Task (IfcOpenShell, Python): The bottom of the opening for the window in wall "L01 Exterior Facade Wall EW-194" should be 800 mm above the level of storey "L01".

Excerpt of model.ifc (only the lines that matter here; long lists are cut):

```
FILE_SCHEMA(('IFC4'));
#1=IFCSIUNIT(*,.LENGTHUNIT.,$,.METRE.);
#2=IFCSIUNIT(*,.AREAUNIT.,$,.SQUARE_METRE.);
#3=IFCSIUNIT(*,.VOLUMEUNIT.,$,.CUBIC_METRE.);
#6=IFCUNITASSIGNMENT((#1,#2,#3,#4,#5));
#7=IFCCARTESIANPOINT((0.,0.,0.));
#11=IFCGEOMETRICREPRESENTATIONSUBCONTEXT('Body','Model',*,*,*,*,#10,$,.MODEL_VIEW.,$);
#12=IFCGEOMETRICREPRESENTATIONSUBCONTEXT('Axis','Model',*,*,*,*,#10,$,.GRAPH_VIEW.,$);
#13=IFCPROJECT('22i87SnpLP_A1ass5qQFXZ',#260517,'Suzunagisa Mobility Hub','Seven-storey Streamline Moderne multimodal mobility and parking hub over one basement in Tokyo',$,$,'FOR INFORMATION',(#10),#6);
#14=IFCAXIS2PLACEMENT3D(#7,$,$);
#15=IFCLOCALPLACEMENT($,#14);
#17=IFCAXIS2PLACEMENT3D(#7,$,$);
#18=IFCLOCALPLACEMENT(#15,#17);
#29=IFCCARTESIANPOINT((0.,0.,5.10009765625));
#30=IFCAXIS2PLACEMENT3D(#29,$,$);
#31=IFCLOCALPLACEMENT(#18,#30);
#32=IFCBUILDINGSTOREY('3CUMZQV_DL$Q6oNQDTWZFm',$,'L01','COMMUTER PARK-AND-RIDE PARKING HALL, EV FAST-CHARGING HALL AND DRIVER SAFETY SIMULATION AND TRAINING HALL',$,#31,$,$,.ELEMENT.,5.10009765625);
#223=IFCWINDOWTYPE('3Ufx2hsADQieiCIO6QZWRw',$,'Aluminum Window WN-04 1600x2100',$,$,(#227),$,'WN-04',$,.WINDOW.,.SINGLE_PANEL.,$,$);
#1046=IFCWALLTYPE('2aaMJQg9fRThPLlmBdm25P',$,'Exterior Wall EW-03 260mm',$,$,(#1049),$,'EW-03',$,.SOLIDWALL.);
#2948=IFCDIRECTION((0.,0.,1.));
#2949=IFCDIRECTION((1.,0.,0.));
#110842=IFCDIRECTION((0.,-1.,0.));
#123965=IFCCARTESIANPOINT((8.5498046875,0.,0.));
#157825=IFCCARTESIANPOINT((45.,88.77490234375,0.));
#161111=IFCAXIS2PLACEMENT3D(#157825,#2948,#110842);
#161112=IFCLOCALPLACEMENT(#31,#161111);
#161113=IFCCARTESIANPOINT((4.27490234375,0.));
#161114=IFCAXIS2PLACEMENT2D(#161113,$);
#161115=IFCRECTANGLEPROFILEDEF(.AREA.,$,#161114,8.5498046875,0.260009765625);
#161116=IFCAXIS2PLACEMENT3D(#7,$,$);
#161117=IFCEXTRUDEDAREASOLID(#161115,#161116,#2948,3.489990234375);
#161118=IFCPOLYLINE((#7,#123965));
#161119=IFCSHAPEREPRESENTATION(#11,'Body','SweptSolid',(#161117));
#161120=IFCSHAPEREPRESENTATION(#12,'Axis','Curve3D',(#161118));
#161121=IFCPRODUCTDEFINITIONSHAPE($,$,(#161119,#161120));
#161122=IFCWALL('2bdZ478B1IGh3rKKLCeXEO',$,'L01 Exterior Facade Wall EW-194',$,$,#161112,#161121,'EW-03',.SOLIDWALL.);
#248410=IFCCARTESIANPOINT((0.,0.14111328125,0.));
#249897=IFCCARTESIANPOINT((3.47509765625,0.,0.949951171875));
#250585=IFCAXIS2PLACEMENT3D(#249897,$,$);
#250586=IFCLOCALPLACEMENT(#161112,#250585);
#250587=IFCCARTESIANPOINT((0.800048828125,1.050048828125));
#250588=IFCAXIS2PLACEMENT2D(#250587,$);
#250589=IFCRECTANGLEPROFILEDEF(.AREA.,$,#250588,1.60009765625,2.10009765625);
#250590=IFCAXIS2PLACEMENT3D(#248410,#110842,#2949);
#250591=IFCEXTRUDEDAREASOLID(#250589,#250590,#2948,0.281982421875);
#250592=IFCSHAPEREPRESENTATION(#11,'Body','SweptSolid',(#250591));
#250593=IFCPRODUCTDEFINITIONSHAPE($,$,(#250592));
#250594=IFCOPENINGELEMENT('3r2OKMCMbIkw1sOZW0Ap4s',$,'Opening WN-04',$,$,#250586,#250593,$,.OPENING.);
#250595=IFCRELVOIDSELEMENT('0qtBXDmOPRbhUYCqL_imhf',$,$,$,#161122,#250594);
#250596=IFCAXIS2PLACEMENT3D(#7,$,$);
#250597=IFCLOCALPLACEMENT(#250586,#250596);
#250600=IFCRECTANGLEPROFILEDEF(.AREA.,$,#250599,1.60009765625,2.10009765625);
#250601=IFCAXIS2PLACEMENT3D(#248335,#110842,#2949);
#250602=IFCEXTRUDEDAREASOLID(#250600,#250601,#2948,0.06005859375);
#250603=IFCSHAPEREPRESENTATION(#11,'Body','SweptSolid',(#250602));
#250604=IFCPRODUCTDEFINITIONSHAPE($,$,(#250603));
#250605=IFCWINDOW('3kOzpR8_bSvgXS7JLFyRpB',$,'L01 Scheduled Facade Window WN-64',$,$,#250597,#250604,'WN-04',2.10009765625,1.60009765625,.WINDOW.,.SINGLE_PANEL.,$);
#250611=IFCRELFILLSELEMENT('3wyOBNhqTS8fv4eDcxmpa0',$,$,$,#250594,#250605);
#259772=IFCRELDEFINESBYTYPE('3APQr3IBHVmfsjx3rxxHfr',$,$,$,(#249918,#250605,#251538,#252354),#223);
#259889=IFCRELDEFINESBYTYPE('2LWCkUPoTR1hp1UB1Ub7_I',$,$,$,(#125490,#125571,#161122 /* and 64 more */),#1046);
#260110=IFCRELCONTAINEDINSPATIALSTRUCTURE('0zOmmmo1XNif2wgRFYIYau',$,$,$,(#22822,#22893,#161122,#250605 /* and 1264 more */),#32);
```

```python
import numpy as np
import ifcopenshell
import ifcopenshell.api.geometry
import ifcopenshell.geom
import ifcopenshell.util.element
import ifcopenshell.util.placement
import ifcopenshell.util.shape
import ifcopenshell.util.unit

model = ifcopenshell.open("model.ifc")
unit_scale = ifcopenshell.util.unit.calculate_unit_scale(model)

window = model.by_id(250605)
opening = window.FillsVoids[0].RelatingOpeningElement
storey = ifcopenshell.util.element.get_container(window, ifc_class="IfcBuildingStorey")
level = ifcopenshell.util.placement.get_local_placement(storey.ObjectPlacement)[2, 3]

# The opening's origin need not be at the sill, so measure its lowest point.
shape = ifcopenshell.geom.create_shape(ifcopenshell.geom.settings(), opening)
bottom = ifcopenshell.util.shape.get_shape_bottom_elevation(shape, shape.geometry) / unit_scale
dz = level + 0.8 / unit_scale - bottom

shift = np.array([0.0, 0.0, dz])
# The window is placed relative to its opening, so it follows when the opening moves.
matrix = ifcopenshell.util.placement.get_local_placement(opening.ObjectPlacement)
matrix[:3, 3] += shift
ifcopenshell.api.geometry.edit_object_placement(
    model, product=opening, matrix=matrix, is_si=False, should_transform_children=True
)

print(f"moved by {dz * unit_scale:+.3f} m")

model.write("model_v2.ifc")
```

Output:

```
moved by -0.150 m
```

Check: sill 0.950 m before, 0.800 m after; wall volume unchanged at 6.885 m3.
